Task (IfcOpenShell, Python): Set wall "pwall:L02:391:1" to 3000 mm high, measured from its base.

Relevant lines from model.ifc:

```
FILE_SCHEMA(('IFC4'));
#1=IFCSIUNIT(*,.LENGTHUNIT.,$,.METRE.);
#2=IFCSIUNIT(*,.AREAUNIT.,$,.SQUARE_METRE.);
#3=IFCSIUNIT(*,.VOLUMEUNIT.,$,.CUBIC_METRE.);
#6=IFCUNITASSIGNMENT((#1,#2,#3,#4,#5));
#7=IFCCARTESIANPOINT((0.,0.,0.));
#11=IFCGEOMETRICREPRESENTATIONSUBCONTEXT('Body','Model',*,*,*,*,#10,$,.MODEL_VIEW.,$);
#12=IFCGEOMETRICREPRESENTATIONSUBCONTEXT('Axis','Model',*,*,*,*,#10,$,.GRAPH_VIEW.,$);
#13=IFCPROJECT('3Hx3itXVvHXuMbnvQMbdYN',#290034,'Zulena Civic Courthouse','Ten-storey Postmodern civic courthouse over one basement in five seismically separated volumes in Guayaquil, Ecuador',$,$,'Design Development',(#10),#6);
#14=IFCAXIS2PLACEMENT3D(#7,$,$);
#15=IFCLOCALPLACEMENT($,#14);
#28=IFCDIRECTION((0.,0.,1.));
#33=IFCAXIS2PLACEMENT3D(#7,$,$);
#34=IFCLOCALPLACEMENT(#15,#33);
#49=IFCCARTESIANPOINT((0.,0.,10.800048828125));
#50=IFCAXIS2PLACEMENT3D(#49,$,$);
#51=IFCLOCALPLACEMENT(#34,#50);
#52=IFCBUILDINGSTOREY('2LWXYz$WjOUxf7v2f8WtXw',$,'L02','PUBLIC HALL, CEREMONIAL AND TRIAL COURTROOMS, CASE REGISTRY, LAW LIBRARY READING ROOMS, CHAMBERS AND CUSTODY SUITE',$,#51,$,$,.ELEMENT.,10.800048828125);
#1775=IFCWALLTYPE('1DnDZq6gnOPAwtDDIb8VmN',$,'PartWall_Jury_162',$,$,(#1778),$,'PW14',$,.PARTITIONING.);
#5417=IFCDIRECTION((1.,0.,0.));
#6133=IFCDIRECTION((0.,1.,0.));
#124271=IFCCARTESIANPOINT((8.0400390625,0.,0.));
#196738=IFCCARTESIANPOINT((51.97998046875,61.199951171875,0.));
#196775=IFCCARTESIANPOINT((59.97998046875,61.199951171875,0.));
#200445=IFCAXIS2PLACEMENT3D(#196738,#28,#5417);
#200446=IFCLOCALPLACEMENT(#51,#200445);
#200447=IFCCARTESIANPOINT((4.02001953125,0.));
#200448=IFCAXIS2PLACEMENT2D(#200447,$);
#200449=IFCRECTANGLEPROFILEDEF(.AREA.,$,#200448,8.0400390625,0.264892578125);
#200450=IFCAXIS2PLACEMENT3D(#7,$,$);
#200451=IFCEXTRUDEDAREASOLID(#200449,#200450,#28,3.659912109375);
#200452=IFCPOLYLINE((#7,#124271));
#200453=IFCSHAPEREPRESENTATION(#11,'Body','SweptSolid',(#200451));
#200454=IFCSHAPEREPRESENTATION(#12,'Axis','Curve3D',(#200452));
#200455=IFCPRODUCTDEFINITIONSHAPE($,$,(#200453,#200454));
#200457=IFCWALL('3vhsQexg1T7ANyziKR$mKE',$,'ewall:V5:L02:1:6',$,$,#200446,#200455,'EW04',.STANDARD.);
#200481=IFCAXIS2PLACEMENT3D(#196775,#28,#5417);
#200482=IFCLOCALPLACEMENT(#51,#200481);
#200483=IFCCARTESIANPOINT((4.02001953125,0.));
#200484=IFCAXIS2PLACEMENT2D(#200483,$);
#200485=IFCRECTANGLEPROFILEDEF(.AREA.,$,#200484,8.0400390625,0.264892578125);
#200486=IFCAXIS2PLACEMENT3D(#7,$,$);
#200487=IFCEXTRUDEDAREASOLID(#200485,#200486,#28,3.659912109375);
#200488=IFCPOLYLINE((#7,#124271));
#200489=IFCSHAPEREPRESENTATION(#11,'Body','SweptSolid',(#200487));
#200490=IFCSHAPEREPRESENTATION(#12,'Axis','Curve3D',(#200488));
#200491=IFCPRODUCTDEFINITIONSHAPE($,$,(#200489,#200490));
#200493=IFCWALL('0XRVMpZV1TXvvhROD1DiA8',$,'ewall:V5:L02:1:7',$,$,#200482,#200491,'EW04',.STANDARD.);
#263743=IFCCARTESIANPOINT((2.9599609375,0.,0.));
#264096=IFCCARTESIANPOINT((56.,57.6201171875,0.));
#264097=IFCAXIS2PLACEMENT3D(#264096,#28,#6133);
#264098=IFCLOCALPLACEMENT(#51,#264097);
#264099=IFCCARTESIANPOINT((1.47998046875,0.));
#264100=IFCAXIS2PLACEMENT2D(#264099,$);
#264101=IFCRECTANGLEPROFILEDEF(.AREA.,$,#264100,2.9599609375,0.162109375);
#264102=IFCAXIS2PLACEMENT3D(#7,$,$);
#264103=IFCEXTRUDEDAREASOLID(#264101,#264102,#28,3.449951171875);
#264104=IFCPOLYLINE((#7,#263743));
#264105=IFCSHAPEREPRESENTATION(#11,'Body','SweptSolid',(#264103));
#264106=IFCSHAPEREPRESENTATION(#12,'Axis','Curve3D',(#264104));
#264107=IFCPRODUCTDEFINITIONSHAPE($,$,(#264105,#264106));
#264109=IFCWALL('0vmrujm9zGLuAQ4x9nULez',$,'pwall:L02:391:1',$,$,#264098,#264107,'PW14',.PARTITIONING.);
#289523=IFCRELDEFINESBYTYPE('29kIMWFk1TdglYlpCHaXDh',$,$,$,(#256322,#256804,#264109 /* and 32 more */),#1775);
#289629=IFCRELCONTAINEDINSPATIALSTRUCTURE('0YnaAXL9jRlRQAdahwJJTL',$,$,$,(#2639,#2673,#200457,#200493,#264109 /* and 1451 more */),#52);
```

```python
import ifcopenshell
import ifcopenshell.geom
import ifcopenshell.util.representation
import ifcopenshell.util.shape

model = ifcopenshell.open("model.ifc")
settings = ifcopenshell.geom.settings()


def volume(element):
    """Net volume in cubic metres, openings subtracted."""
    shape = ifcopenshell.geom.create_shape(settings, element)
    return ifcopenshell.util.shape.get_volume(shape.geometry)


wall = model.by_guid("0vmrujm9zGLuAQ4x9nULez")
before = volume(wall)

body = ifcopenshell.util.representation.get_representation(wall, "Model", "Body")
solid = body.Items[0]
old_height = solid.Depth
solid.Depth = 3.0
after = volume(wall)

print(f"height {old_height:g} -> {solid.Depth:g}, volume {before:.3f} -> {after:.3f} m3")

model.write("model_edited.ifc")
```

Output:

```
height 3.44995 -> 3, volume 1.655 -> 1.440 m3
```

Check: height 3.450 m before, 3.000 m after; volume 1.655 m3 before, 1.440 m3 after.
